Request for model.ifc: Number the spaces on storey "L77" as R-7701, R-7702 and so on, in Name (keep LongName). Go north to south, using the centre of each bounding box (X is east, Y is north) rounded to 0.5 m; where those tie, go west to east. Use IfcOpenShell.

First a look at what the model holds.

```python
import ifcopenshell
import ifcopenshell.util.element
import ifcopenshell.util.placement

model = ifcopenshell.open("model.ifc")
print(model.schema)
storey = next(s for s in model.by_type("IfcBuildingStorey") if s.Name == "L77")
spaces = [e for e in ifcopenshell.util.element.get_decomposition(storey) if e.is_a("IfcSpace")]
for e in sorted(spaces, key=lambda e: e.id()):
    origin = ifcopenshell.util.placement.get_local_placement(e.ObjectPlacement)[:3, 3]
    print(e.id(), e.Name, e.LongName, origin.round(2) + 0.0, sep=" | ")
```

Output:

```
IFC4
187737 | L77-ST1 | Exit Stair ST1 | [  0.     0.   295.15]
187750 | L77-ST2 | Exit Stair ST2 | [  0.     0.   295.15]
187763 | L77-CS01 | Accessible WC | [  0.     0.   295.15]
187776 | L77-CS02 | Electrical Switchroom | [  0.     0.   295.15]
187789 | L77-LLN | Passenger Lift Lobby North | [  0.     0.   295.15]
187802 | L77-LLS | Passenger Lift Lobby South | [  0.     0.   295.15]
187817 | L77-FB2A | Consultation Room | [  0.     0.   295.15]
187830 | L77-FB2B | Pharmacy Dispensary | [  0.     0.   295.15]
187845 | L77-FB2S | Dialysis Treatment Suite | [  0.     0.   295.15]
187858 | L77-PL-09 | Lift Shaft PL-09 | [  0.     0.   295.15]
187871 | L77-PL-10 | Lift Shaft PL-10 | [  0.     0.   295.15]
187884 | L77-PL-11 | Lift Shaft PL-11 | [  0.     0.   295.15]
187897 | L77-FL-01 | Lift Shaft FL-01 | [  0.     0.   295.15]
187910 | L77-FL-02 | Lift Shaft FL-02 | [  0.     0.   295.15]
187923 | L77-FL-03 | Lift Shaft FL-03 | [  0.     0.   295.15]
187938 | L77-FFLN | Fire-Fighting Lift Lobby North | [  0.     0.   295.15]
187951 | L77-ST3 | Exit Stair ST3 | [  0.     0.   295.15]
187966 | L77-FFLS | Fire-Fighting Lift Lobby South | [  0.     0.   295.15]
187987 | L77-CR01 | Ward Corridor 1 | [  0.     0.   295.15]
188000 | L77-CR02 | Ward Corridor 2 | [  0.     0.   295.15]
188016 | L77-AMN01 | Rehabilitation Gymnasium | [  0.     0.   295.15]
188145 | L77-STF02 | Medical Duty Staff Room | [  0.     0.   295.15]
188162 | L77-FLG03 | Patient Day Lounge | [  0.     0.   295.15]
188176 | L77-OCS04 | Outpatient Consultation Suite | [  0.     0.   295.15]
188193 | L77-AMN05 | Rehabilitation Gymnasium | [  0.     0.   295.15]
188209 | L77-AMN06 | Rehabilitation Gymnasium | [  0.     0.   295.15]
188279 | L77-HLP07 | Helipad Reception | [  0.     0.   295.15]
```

```python
import ifcopenshell
import ifcopenshell.geom
import ifcopenshell.util.element
import ifcopenshell.util.shape

model = ifcopenshell.open("model.ifc")
settings = ifcopenshell.geom.settings()
settings.set("use-world-coords", True)


def centre(element):
    shape = ifcopenshell.geom.create_shape(settings, element)
    return ifcopenshell.util.shape.get_bbox_centroid(shape.geometry)


storey = next(s for s in model.by_type("IfcBuildingStorey") if s.Name == "L77")
spaces = [e for e in ifcopenshell.util.element.get_decomposition(storey) if e.is_a("IfcSpace")]

# Insertion points can sit at a corner or the storey origin, so sort by the geometry (in metres).
centres = {e: centre(e) for e in spaces}
spaces.sort(key=lambda e: (-round(centres[e][1] / 0.5), centres[e][0]))

for i, e in enumerate(spaces, start=1):
    number = f"R-77{i:02d}"
    e.Name = number
    print(e.id(), number)

model.write("model_v2.ifc")
```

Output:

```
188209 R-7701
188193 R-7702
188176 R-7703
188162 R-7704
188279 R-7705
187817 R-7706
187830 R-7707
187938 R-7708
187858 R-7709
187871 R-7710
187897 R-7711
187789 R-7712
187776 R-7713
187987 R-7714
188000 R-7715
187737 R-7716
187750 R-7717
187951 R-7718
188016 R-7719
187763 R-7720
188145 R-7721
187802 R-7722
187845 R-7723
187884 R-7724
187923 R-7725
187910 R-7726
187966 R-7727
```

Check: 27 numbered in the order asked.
